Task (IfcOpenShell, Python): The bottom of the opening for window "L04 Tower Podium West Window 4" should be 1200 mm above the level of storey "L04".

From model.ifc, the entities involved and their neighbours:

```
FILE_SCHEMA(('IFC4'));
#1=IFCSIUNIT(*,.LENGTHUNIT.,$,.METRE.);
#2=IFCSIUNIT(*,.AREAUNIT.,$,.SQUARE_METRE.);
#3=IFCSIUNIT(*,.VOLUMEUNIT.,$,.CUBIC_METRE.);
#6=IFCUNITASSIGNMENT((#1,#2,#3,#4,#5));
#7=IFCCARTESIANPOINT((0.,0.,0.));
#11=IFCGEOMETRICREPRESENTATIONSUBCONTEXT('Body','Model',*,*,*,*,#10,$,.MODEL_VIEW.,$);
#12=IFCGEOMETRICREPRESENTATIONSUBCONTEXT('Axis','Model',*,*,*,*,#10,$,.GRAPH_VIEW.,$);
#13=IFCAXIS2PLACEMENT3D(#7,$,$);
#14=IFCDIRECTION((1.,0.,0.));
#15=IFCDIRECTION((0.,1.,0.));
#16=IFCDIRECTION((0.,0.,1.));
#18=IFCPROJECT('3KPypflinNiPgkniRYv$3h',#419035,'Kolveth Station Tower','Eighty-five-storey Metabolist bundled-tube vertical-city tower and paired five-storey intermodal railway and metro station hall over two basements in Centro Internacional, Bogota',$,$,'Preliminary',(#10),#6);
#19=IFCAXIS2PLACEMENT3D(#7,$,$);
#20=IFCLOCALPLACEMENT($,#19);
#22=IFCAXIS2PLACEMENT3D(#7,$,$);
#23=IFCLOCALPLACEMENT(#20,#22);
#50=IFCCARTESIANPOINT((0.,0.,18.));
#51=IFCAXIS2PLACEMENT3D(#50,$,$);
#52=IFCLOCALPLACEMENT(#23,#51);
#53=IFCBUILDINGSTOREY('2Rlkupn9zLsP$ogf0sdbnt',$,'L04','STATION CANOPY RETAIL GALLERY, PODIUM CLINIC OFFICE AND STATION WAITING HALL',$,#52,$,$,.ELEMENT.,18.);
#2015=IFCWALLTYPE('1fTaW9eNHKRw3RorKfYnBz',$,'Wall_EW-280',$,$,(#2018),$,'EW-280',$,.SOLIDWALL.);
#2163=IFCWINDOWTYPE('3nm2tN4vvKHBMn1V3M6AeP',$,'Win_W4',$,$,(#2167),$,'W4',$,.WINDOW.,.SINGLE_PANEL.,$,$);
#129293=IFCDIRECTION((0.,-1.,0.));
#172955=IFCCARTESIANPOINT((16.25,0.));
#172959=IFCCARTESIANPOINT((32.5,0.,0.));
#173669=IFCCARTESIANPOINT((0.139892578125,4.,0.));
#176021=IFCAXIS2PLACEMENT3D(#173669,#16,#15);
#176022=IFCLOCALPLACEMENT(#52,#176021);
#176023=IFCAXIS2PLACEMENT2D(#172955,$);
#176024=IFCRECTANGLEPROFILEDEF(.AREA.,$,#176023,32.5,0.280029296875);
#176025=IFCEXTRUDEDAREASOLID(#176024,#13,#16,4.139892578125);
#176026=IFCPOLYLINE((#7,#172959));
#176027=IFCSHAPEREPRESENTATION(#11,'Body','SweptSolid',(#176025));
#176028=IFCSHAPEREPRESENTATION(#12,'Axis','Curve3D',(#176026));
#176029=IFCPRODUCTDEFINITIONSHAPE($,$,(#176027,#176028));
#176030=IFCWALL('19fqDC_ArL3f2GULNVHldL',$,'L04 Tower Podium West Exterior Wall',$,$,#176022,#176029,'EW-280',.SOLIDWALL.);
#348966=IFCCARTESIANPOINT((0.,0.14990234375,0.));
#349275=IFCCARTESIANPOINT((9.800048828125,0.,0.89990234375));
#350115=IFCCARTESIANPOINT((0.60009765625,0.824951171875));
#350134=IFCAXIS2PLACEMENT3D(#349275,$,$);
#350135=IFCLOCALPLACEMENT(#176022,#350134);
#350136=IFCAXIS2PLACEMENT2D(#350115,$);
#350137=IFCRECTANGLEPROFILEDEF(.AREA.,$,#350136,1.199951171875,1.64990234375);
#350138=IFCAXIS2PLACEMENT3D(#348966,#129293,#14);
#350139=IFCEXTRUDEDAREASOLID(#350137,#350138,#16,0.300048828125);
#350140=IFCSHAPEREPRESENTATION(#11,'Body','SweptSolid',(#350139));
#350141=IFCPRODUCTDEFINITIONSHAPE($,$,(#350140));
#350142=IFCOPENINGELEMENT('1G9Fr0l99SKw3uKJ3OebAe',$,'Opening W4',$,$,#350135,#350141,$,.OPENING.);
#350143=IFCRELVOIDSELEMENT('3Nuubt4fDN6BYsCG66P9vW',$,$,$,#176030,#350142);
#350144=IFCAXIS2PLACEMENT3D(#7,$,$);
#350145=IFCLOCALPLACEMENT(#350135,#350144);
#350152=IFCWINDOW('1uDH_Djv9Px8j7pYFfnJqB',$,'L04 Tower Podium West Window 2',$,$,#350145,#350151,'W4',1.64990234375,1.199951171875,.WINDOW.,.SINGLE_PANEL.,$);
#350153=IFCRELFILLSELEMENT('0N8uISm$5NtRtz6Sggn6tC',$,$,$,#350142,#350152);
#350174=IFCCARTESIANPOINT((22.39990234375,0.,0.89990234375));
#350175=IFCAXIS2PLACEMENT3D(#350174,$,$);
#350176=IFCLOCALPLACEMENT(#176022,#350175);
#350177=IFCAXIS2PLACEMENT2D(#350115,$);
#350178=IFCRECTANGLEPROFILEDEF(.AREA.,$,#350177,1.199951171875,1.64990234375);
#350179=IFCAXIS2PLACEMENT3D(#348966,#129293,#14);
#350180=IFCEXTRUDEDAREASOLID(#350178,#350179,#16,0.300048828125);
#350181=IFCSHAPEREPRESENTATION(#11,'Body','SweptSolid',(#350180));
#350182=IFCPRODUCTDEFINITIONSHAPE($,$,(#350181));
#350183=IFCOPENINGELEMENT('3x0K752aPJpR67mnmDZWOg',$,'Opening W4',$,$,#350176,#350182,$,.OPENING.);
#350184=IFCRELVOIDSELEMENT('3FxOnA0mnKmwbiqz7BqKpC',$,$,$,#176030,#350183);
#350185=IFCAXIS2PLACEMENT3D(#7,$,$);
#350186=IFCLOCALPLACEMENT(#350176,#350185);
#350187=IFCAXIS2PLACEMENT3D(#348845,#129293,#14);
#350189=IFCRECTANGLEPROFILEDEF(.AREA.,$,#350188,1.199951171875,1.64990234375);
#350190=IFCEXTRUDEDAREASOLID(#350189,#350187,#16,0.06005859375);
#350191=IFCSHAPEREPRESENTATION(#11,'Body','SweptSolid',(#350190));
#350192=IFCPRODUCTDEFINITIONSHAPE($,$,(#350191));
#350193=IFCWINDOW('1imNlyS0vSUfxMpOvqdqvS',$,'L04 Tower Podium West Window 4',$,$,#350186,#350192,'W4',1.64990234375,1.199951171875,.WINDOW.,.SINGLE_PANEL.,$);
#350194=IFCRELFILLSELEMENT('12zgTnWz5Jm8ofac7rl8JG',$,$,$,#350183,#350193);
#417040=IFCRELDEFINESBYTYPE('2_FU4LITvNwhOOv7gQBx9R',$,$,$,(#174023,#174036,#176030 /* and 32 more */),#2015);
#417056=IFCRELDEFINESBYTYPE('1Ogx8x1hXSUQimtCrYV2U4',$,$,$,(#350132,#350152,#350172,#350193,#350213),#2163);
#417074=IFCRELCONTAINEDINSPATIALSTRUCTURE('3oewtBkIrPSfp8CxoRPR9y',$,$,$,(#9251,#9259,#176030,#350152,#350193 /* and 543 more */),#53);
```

```python
import numpy as np
import ifcopenshell
import ifcopenshell.api.geometry
import ifcopenshell.geom
import ifcopenshell.util.element
import ifcopenshell.util.placement
import ifcopenshell.util.shape
import ifcopenshell.util.unit

model = ifcopenshell.open("model.ifc")
unit_scale = ifcopenshell.util.unit.calculate_unit_scale(model)

window = model.by_guid("1imNlyS0vSUfxMpOvqdqvS")
opening = window.FillsVoids[0].RelatingOpeningElement
storey = ifcopenshell.util.element.get_container(window, ifc_class="IfcBuildingStorey")
level = ifcopenshell.util.placement.get_local_placement(storey.ObjectPlacement)[2, 3]

# The opening's origin need not be at the sill, so measure its lowest point.
shape = ifcopenshell.geom.create_shape(ifcopenshell.geom.settings(), opening)
bottom = ifcopenshell.util.shape.get_shape_bottom_elevation(shape, shape.geometry) / unit_scale
dz = level + 1.2 / unit_scale - bottom

shift = np.array([0.0, 0.0, dz])
# The window is placed relative to its opening, so it follows when the opening moves.
matrix = ifcopenshell.util.placement.get_local_placement(opening.ObjectPlacement)
matrix[:3, 3] += shift
ifcopenshell.api.geometry.edit_object_placement(
    model, product=opening, matrix=matrix, is_si=False, should_transform_children=True
)

print(f"moved by {dz * unit_scale:+.3f} m")

model.write("model_rev.ifc")
```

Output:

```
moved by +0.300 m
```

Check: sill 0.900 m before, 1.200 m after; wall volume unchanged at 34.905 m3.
